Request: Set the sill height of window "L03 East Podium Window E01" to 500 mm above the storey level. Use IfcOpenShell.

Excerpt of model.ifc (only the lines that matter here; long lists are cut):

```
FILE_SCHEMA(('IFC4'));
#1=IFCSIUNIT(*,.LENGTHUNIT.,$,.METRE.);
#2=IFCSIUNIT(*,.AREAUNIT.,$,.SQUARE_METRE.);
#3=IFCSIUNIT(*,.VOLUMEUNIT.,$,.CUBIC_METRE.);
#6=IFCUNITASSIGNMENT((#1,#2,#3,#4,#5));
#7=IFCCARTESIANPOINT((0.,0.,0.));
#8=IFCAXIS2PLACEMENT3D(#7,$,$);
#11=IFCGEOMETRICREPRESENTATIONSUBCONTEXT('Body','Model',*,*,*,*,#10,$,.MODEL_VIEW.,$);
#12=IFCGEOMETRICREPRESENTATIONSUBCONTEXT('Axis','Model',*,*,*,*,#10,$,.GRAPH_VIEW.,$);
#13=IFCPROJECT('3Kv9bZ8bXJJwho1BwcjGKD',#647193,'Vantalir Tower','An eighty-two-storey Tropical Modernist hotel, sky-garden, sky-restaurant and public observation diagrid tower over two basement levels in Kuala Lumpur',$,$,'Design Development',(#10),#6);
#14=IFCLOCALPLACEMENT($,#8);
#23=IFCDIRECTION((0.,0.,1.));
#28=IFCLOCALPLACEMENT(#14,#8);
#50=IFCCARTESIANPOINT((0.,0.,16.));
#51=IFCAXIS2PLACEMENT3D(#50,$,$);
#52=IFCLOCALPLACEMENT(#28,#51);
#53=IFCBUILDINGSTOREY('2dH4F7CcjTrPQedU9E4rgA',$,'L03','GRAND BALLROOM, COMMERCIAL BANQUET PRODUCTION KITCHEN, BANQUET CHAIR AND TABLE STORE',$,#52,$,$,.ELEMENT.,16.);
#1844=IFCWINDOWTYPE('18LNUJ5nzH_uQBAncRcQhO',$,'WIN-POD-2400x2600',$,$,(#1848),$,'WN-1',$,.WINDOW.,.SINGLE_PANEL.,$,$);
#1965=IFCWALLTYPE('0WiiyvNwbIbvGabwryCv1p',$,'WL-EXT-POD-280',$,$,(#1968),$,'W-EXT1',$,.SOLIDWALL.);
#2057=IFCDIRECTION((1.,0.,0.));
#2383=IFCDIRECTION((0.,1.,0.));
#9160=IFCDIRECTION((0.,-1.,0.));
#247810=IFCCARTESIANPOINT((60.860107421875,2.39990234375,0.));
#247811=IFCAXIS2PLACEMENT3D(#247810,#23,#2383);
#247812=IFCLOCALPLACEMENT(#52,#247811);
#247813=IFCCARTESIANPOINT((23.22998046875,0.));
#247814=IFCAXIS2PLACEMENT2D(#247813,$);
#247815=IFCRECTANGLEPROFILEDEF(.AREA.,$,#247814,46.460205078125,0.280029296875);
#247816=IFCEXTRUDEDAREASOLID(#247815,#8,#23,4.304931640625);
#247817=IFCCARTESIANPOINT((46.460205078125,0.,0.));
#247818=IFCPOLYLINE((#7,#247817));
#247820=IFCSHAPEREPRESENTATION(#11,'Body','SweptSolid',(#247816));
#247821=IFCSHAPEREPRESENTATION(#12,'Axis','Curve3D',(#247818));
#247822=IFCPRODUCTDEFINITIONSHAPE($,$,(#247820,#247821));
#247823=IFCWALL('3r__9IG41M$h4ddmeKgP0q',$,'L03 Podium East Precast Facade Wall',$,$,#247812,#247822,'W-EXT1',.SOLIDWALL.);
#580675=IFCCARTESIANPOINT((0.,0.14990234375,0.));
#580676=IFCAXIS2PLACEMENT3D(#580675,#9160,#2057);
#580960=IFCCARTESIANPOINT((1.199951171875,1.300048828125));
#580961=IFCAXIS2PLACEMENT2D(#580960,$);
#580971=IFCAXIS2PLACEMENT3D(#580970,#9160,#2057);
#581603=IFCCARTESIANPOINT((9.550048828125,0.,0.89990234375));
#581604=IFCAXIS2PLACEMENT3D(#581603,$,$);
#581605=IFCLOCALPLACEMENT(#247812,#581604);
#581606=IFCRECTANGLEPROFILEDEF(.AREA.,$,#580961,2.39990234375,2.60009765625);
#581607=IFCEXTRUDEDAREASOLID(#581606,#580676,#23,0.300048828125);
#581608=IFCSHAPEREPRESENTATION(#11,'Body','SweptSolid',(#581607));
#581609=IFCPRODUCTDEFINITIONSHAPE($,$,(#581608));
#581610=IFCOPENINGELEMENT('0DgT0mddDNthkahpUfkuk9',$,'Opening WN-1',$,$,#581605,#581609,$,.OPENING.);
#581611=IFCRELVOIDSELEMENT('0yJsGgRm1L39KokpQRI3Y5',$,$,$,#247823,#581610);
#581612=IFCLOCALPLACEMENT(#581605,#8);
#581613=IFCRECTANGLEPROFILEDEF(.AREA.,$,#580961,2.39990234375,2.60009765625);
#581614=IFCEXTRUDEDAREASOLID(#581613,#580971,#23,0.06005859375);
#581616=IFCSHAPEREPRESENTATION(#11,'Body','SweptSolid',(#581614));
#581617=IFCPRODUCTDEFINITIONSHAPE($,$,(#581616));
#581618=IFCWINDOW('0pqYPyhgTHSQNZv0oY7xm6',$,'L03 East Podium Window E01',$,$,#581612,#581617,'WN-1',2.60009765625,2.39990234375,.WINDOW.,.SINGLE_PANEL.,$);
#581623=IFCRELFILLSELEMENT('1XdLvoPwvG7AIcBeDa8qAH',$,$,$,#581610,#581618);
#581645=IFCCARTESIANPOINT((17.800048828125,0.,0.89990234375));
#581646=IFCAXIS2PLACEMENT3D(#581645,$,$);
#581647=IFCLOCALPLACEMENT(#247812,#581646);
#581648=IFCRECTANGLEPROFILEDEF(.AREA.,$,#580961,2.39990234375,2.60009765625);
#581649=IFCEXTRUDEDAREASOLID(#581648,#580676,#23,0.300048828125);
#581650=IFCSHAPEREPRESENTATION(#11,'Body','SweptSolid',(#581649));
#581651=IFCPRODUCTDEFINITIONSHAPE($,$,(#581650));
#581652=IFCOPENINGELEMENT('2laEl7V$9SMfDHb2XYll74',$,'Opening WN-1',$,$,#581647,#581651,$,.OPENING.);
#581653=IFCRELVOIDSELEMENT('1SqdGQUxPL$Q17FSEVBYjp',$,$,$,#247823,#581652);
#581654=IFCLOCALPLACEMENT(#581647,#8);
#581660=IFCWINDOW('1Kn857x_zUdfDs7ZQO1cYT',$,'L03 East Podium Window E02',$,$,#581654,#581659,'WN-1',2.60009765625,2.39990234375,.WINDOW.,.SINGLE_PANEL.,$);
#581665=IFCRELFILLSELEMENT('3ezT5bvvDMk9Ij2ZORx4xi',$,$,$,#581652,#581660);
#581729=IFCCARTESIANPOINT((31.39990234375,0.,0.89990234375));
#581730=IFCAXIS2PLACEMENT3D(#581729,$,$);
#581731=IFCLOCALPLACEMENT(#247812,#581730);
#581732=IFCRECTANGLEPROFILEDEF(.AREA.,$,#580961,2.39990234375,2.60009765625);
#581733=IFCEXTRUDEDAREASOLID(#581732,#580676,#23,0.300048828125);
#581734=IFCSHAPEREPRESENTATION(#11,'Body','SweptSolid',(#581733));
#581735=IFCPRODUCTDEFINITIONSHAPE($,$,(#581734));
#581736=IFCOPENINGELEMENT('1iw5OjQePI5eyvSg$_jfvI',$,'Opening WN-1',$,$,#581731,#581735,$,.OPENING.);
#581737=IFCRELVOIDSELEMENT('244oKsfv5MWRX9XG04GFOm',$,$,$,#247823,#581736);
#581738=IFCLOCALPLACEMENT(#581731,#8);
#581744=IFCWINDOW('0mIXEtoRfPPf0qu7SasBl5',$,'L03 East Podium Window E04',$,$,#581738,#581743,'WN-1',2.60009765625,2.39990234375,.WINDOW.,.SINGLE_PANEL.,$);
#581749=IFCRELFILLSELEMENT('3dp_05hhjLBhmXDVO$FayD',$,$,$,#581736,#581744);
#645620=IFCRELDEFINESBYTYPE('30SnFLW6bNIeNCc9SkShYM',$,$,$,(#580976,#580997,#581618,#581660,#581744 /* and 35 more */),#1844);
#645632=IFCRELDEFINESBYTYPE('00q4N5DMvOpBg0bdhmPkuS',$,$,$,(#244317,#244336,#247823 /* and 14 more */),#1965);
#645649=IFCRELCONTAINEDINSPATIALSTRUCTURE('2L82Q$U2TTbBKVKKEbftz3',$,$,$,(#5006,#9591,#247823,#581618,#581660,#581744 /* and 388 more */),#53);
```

```python
import numpy as np
import ifcopenshell
import ifcopenshell.api.geometry
import ifcopenshell.geom
import ifcopenshell.util.element
import ifcopenshell.util.placement
import ifcopenshell.util.shape
import ifcopenshell.util.unit

model = ifcopenshell.open("model.ifc")
unit_scale = ifcopenshell.util.unit.calculate_unit_scale(model)

window = model.by_guid("0pqYPyhgTHSQNZv0oY7xm6")
opening = window.FillsVoids[0].RelatingOpeningElement
storey = ifcopenshell.util.element.get_container(window, ifc_class="IfcBuildingStorey")
level = ifcopenshell.util.placement.get_local_placement(storey.ObjectPlacement)[2, 3]

# The opening's origin need not be at the sill, so measure its lowest point.
shape = ifcopenshell.geom.create_shape(ifcopenshell.geom.settings(), opening)
bottom = ifcopenshell.util.shape.get_shape_bottom_elevation(shape, shape.geometry) / unit_scale
dz = level + 0.5 / unit_scale - bottom

shift = np.array([0.0, 0.0, dz])
# The window is placed relative to its opening, so it follows when the opening moves.
matrix = ifcopenshell.util.placement.get_local_placement(opening.ObjectPlacement)
matrix[:3, 3] += shift
ifcopenshell.api.geometry.edit_object_placement(
    model, product=opening, matrix=matrix, is_si=False, should_transform_children=True
)

print(f"moved by {dz * unit_scale:+.3f} m")

model.write("model_updated.ifc")
```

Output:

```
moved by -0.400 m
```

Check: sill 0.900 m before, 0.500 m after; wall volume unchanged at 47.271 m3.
